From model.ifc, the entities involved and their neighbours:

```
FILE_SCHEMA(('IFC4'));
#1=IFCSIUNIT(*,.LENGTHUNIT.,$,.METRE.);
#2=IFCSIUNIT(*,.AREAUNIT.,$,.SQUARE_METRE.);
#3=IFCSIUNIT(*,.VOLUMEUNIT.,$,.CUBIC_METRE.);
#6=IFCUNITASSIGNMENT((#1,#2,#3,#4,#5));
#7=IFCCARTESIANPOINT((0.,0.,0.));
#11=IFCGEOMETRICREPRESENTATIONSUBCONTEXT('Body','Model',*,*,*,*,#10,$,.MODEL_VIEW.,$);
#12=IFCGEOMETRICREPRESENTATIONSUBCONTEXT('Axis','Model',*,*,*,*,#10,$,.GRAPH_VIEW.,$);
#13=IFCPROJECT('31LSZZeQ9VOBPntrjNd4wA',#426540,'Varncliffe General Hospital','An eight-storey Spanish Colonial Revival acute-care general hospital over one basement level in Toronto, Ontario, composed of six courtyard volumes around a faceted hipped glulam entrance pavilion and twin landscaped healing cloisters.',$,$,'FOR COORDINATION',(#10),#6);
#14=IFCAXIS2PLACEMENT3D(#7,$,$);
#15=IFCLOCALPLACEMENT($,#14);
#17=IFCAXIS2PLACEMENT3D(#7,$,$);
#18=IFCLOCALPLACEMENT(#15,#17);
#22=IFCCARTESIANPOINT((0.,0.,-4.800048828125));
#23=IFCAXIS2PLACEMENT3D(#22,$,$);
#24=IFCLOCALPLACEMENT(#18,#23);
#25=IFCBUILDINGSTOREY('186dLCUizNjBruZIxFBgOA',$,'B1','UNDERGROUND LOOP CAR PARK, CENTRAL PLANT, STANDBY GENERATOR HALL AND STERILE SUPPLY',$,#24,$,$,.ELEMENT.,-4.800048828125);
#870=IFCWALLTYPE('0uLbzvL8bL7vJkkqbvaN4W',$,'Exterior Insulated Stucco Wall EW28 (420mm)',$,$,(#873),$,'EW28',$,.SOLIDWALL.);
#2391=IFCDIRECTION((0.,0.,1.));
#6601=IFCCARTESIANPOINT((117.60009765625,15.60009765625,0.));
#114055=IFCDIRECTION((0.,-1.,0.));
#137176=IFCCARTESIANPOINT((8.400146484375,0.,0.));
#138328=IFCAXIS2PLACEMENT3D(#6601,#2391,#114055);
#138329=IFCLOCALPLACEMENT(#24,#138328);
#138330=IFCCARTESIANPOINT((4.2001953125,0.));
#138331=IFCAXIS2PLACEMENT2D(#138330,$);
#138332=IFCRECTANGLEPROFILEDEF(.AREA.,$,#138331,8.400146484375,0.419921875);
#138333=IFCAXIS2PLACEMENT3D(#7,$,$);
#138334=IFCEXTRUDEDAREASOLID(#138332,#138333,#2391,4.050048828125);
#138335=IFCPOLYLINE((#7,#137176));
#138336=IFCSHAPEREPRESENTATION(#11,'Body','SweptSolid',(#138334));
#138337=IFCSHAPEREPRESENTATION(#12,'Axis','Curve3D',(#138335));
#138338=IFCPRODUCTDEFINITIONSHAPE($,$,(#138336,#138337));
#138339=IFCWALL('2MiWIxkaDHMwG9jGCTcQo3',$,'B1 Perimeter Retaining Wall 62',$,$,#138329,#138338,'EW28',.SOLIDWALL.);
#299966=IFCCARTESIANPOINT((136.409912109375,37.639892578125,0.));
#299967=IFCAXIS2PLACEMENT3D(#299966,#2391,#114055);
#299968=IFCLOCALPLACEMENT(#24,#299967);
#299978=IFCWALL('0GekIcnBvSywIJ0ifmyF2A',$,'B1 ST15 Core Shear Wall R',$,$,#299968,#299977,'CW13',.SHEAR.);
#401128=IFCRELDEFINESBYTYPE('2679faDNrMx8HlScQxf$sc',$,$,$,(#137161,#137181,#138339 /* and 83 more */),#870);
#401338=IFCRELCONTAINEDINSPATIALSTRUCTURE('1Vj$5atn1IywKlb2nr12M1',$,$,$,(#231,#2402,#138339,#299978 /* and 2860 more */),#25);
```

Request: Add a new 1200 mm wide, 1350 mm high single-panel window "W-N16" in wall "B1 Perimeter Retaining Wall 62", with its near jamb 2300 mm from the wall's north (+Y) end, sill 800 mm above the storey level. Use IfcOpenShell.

```python
import numpy as np
import ifcopenshell
import ifcopenshell.api.feature
import ifcopenshell.api.geometry
import ifcopenshell.api.root
import ifcopenshell.api.spatial
import ifcopenshell.geom
import ifcopenshell.util.element
import ifcopenshell.util.placement
import ifcopenshell.util.representation
import ifcopenshell.util.shape
import ifcopenshell.util.unit

model = ifcopenshell.open("model.ifc")
unit_scale = ifcopenshell.util.unit.calculate_unit_scale(model)
settings = ifcopenshell.geom.settings()


def volume(element):
    """Net volume in cubic metres, openings subtracted."""
    shape = ifcopenshell.geom.create_shape(settings, element)
    return ifcopenshell.util.shape.get_volume(shape.geometry)


wall = model.by_id(138339)
storey = ifcopenshell.util.element.get_container(wall, ifc_class="IfcBuildingStorey")
context = ifcopenshell.util.representation.get_context(model, "Model", "Body", "MODEL_VIEW")
before = volume(wall)

width, height, from_end, sill = 1.2, 1.35, 2.3, 0.8  # metres

# The wall runs along its own X axis, and the end named is its -X end.
wall_shape = ifcopenshell.geom.create_shape(settings, wall)
x, y, z = ifcopenshell.util.shape.get_vertices(wall_shape.geometry).T
start = x.min() + from_end
face, thickness = float(y.min()), float(y.max() - y.min())
wall_matrix = ifcopenshell.util.placement.get_local_placement(wall.ObjectPlacement)
level = ifcopenshell.util.placement.get_local_placement(storey.ObjectPlacement)[2, 3]


def in_wall(x, y):
    """Placement at x, y metres in the wall's axes, at sill height."""
    matrix = wall_matrix.copy()
    matrix[:, 3] = wall_matrix @ np.array([x / unit_scale, y / unit_scale, 0.0, 1.0])
    matrix[2, 3] = level + sill / unit_scale
    return matrix


# Opening: a box that overshoots both wall faces by 50 mm.
opening = ifcopenshell.api.root.create_entity(model, ifc_class="IfcOpeningElement", predefined_type="OPENING")
box = ifcopenshell.api.geometry.add_wall_representation(
    model, context=context, length=width, height=height, thickness=thickness + 0.1
)
ifcopenshell.api.geometry.assign_representation(model, product=opening, representation=box)
ifcopenshell.api.geometry.edit_object_placement(model, product=opening, matrix=in_wall(start, face - 0.05), is_si=False)
ifcopenshell.api.feature.add_feature(model, feature=opening, element=wall)

window = ifcopenshell.api.root.create_entity(model, ifc_class="IfcWindow", name="W-N16", predefined_type="WINDOW")
window.OverallWidth, window.OverallHeight = width / unit_scale, height / unit_scale
window.PartitioningType = "SINGLE_PANEL"
body = ifcopenshell.api.geometry.add_window_representation(
    model,
    context=context,
    overall_width=window.OverallWidth,
    overall_height=window.OverallHeight,
    partition_type="SINGLE_PANEL",
)
ifcopenshell.api.geometry.assign_representation(model, product=window, representation=body)
ifcopenshell.api.spatial.assign_container(model, products=[window], relating_structure=storey)
ifcopenshell.api.feature.add_filling(model, opening=opening, element=window)

# Centre the window in the wall's thickness.
ifcopenshell.api.geometry.edit_object_placement(model, product=window, matrix=in_wall(start, face), is_si=False)
window_shape = ifcopenshell.geom.create_shape(settings, window)
depth = ifcopenshell.util.shape.get_vertices(window_shape.geometry)[:, 1]
offset = face + thickness / 2 - (depth.min() + depth.max()) / 2
ifcopenshell.api.geometry.edit_object_placement(model, product=window, matrix=in_wall(start, offset), is_si=False)

after = volume(wall)

print(f"wall volume {before:.3f} -> {after:.3f} m3")

model.write("model_updated.ifc")
```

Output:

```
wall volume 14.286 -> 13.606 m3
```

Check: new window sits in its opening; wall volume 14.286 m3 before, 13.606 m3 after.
